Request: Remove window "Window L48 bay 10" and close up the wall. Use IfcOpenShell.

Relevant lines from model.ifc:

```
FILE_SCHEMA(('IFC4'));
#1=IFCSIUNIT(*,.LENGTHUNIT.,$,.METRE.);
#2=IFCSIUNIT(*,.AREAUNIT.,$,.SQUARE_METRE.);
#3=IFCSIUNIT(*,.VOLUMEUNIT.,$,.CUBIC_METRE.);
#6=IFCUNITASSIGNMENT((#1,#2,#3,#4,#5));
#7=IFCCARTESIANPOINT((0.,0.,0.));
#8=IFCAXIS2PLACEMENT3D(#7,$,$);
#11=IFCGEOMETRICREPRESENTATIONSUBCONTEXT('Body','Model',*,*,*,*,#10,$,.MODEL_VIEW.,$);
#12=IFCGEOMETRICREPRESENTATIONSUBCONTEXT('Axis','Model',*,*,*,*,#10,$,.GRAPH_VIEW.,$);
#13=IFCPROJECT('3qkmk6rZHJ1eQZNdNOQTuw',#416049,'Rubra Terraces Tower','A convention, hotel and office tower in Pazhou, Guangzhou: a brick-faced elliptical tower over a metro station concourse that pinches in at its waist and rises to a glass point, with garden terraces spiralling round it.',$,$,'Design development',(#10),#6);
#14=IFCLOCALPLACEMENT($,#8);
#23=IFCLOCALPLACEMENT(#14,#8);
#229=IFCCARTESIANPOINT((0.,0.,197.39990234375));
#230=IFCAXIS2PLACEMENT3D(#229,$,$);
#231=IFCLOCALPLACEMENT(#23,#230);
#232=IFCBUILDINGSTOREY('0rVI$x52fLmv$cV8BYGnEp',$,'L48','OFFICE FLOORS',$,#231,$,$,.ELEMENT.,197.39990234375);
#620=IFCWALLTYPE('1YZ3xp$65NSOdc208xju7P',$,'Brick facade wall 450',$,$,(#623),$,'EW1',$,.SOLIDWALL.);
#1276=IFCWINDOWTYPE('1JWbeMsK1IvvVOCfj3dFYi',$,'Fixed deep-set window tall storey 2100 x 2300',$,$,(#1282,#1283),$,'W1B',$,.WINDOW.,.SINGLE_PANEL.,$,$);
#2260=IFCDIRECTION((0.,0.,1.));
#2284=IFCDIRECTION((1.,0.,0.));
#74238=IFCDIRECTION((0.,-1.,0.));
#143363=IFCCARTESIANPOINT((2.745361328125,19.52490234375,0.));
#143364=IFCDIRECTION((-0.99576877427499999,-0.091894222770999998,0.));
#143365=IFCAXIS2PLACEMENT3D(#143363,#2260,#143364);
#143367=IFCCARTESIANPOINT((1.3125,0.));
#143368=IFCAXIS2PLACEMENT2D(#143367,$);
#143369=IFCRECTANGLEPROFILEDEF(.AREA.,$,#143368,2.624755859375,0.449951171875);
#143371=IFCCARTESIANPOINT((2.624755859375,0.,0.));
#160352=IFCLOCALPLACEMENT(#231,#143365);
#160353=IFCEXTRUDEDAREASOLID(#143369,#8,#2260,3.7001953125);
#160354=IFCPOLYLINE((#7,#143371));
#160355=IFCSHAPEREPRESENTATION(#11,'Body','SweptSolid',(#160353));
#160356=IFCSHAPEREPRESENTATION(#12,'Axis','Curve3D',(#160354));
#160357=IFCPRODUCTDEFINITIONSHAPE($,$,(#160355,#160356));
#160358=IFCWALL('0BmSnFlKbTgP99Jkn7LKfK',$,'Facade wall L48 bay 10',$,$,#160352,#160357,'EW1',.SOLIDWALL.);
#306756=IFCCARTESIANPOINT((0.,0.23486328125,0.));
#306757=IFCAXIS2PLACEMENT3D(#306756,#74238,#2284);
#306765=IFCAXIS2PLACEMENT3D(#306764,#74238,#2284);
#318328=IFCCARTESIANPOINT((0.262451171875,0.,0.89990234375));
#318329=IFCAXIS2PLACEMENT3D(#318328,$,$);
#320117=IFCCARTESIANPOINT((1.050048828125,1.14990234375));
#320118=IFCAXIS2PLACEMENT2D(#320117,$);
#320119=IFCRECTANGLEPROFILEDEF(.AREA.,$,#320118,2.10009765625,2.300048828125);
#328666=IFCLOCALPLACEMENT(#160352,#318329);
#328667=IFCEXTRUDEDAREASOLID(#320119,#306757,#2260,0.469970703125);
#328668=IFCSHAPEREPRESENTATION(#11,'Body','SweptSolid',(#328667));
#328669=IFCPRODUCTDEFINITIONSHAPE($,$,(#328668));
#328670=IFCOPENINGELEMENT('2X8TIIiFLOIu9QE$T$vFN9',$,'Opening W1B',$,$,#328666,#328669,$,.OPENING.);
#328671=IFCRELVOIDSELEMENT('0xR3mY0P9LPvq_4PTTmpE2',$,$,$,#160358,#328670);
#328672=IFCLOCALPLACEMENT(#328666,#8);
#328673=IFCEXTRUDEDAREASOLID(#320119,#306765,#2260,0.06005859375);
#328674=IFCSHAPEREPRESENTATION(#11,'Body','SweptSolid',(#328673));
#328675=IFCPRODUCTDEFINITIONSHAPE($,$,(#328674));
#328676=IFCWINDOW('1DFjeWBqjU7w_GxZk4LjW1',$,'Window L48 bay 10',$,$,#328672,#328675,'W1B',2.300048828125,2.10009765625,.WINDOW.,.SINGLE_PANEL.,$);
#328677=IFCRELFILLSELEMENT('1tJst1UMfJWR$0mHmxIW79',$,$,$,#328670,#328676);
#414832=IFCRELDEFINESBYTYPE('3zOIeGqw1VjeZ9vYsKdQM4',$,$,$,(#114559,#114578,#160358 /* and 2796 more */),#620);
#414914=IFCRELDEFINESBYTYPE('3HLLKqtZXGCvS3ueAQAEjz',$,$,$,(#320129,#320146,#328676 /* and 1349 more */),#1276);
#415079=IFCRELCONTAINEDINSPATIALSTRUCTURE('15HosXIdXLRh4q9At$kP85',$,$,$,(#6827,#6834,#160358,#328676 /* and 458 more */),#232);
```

```python
import ifcopenshell
import ifcopenshell.api.feature
import ifcopenshell.api.root
import ifcopenshell.geom
import ifcopenshell.util.shape

model = ifcopenshell.open("model.ifc")
settings = ifcopenshell.geom.settings()


def volume(element):
    """Net volume in cubic metres, openings subtracted."""
    shape = ifcopenshell.geom.create_shape(settings, element)
    return ifcopenshell.util.shape.get_volume(shape.geometry)


window = model.by_id(328676)
opening = window.FillsVoids[0].RelatingOpeningElement
wall = opening.VoidsElements[0].RelatingBuildingElement
before = volume(wall)

ifcopenshell.api.root.remove_product(model, product=window)
ifcopenshell.api.feature.remove_feature(model, feature=opening)

after = volume(wall)

print(f"wall volume {before:.3f} -> {after:.3f} m3")

model.write("model_v2.ifc")
```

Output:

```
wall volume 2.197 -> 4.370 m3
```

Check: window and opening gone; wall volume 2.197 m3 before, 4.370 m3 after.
